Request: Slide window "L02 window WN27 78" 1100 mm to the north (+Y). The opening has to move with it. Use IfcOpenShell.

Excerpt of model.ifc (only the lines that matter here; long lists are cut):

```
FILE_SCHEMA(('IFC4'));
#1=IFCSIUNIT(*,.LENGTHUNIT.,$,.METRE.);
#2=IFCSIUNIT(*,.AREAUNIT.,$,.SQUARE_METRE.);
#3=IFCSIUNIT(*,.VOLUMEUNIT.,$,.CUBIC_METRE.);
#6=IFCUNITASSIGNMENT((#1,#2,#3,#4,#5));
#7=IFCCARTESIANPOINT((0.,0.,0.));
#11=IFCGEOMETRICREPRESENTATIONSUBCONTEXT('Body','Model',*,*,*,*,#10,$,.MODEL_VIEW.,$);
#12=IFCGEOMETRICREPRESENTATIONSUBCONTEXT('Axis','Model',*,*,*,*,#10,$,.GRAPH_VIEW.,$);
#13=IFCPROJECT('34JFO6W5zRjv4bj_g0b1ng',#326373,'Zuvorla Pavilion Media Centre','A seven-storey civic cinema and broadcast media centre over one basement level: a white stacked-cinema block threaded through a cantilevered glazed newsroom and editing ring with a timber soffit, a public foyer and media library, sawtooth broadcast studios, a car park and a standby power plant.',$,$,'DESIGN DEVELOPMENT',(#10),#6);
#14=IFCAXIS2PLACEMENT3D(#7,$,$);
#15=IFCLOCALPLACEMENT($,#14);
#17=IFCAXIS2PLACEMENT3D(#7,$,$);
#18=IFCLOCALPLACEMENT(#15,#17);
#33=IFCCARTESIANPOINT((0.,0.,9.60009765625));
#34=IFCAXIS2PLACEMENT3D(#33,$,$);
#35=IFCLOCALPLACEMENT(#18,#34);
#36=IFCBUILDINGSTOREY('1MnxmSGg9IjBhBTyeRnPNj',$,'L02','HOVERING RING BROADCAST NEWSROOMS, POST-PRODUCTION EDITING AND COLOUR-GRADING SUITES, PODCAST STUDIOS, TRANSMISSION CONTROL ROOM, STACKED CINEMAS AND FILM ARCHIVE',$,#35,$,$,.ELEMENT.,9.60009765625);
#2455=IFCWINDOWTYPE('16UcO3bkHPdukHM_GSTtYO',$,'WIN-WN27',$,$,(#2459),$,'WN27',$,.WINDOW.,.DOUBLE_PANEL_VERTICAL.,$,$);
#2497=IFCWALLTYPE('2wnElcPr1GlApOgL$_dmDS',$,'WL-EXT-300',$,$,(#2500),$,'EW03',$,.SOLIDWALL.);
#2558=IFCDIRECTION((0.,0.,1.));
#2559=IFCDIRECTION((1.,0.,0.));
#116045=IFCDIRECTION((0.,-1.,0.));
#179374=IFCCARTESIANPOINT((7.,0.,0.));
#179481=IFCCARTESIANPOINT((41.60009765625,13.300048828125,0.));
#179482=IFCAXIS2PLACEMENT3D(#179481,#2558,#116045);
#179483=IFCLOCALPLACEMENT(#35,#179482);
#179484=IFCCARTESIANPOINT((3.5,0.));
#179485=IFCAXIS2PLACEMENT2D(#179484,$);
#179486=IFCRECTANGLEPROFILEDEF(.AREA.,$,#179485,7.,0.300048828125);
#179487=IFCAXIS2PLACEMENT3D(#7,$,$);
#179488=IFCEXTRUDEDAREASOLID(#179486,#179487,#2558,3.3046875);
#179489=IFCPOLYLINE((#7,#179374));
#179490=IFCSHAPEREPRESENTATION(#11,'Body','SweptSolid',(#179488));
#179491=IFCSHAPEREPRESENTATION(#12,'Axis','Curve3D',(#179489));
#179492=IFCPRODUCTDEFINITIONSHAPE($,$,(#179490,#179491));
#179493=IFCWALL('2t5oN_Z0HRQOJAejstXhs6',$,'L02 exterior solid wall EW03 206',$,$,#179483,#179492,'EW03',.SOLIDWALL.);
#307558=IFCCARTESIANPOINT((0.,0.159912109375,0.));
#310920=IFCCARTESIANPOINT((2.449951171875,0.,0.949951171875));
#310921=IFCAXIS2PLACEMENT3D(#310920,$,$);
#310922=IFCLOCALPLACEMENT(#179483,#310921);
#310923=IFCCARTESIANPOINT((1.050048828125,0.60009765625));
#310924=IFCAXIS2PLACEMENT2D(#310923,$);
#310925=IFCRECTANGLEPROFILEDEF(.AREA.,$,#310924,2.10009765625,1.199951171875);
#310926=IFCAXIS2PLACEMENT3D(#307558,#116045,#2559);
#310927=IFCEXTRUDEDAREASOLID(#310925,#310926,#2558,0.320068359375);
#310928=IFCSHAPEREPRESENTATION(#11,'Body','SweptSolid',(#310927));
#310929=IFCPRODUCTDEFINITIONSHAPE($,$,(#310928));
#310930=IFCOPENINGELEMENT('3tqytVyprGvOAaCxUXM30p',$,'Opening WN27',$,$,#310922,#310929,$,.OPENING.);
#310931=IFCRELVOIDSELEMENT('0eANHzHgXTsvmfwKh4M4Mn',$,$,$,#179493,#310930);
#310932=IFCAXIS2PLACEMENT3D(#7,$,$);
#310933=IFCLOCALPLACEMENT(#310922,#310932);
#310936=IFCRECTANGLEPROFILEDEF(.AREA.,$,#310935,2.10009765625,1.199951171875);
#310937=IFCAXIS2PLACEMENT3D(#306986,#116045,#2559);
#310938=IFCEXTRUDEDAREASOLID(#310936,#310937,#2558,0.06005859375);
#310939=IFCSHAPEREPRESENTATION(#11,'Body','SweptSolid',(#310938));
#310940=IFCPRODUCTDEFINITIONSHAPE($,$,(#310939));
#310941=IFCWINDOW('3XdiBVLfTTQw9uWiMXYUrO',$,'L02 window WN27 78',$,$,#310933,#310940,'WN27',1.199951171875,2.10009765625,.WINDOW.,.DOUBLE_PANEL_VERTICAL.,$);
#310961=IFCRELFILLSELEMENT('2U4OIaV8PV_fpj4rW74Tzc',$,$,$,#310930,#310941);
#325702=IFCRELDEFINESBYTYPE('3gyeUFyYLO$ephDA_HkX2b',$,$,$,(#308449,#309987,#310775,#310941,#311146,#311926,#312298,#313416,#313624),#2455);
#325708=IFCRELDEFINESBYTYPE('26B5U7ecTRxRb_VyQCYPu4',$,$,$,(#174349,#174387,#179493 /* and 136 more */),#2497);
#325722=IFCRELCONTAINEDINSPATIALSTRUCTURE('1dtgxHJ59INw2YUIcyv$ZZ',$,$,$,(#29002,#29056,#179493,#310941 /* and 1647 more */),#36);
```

```python
import ifcopenshell
import ifcopenshell.api.geometry
import ifcopenshell.util.placement
import ifcopenshell.util.unit

model = ifcopenshell.open("model.ifc")
unit_scale = ifcopenshell.util.unit.calculate_unit_scale(model)

window = model.by_id(310941)
opening = window.FillsVoids[0].RelatingOpeningElement
wall = opening.VoidsElements[0].RelatingBuildingElement

wall_matrix = ifcopenshell.util.placement.get_local_placement(wall.ObjectPlacement)
shift = wall_matrix[:3, 0] * -1.1 / unit_scale
before = ifcopenshell.util.placement.get_local_placement(window.ObjectPlacement)[:3, 3].copy()

# The window is placed relative to its opening, so it follows when the opening moves.
matrix = ifcopenshell.util.placement.get_local_placement(opening.ObjectPlacement)
matrix[:3, 3] += shift
ifcopenshell.api.geometry.edit_object_placement(
    model, product=opening, matrix=matrix, is_si=False, should_transform_children=True
)

after = ifcopenshell.util.placement.get_local_placement(window.ObjectPlacement)[:3, 3]
print("window moved by", (after - before).round(3) + 0.0)

model.write("model_rev.ifc")
```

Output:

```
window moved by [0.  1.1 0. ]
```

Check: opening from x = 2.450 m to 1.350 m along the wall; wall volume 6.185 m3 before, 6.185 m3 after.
